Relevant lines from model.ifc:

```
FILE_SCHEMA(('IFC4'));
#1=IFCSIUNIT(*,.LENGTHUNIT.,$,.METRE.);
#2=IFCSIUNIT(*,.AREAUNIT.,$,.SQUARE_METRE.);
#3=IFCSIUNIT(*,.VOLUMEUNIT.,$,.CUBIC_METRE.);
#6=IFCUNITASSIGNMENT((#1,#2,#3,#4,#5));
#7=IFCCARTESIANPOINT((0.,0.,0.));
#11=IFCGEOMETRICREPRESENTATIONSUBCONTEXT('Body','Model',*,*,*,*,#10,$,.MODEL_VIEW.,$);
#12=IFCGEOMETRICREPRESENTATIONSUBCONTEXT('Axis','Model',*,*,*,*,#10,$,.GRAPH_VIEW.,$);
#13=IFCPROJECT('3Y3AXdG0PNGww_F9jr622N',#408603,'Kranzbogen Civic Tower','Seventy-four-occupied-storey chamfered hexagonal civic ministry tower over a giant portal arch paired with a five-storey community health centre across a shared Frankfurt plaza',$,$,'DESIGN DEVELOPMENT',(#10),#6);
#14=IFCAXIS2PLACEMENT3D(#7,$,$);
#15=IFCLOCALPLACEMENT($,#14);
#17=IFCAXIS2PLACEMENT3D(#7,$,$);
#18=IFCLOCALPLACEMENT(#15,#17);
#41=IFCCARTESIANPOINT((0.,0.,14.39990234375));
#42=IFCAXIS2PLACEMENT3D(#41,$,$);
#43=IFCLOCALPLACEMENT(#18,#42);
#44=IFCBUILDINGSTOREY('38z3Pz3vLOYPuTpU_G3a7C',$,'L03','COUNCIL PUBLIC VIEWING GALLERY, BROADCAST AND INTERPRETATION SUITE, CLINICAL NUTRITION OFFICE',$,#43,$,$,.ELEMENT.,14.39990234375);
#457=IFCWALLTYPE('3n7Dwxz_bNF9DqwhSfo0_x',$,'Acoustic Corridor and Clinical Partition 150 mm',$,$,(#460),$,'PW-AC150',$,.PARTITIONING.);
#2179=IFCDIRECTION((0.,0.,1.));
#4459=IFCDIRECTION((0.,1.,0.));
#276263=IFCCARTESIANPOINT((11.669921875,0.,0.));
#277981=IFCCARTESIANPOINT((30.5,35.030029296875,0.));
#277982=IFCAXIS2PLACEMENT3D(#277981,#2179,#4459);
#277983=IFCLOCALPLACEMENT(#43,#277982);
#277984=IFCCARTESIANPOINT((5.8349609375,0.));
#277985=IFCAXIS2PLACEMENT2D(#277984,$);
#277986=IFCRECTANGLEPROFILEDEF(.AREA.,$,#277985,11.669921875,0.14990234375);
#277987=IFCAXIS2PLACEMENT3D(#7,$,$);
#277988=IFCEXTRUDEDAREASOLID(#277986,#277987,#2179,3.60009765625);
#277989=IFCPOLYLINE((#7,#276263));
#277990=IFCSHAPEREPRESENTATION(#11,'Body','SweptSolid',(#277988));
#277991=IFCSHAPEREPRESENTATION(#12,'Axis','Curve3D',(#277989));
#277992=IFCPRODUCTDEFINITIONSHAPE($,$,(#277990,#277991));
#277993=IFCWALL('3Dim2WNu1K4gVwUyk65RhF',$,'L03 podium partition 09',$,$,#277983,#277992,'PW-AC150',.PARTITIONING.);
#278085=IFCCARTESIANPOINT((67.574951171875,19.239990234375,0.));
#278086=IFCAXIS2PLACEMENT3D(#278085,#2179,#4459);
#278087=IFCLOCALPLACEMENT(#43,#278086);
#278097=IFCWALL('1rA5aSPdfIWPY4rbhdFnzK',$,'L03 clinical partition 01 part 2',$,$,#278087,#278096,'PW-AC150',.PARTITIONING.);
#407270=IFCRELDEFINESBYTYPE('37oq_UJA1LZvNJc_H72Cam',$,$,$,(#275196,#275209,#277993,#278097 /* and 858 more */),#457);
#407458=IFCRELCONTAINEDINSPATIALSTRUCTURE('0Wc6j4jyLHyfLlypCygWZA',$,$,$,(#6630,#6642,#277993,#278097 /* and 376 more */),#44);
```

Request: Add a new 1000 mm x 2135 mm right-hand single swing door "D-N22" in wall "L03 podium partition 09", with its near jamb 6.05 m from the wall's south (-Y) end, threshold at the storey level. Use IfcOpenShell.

```python
import numpy as np
import ifcopenshell
import ifcopenshell.api.feature
import ifcopenshell.api.geometry
import ifcopenshell.api.root
import ifcopenshell.api.spatial
import ifcopenshell.geom
import ifcopenshell.util.element
import ifcopenshell.util.placement
import ifcopenshell.util.representation
import ifcopenshell.util.shape
import ifcopenshell.util.unit

model = ifcopenshell.open("model.ifc")
unit_scale = ifcopenshell.util.unit.calculate_unit_scale(model)
settings = ifcopenshell.geom.settings()


def volume(element):
    """Net volume in cubic metres, openings subtracted."""
    shape = ifcopenshell.geom.create_shape(settings, element)
    return ifcopenshell.util.shape.get_volume(shape.geometry)


wall = model.by_guid("3Dim2WNu1K4gVwUyk65RhF")
storey = ifcopenshell.util.element.get_container(wall, ifc_class="IfcBuildingStorey")
context = ifcopenshell.util.representation.get_context(model, "Model", "Body", "MODEL_VIEW")
before = volume(wall)

width, height, from_end, sill = 1, 2.135, 6.05, 0.0  # metres

# The wall runs along its own X axis, and the end named is its -X end.
wall_shape = ifcopenshell.geom.create_shape(settings, wall)
x, y, z = ifcopenshell.util.shape.get_vertices(wall_shape.geometry).T
start = x.min() + from_end
face, thickness = float(y.min()), float(y.max() - y.min())
wall_matrix = ifcopenshell.util.placement.get_local_placement(wall.ObjectPlacement)
level = ifcopenshell.util.placement.get_local_placement(storey.ObjectPlacement)[2, 3]


def in_wall(x, y):
    """Placement at x, y metres in the wall's axes, at sill height."""
    matrix = wall_matrix.copy()
    matrix[:, 3] = wall_matrix @ np.array([x / unit_scale, y / unit_scale, 0.0, 1.0])
    matrix[2, 3] = level + sill / unit_scale
    return matrix


# Opening: a box that overshoots both wall faces by 50 mm.
opening = ifcopenshell.api.root.create_entity(model, ifc_class="IfcOpeningElement", predefined_type="OPENING")
box = ifcopenshell.api.geometry.add_wall_representation(
    model, context=context, length=width, height=height, thickness=thickness + 0.1
)
ifcopenshell.api.geometry.assign_representation(model, product=opening, representation=box)
ifcopenshell.api.geometry.edit_object_placement(model, product=opening, matrix=in_wall(start, face - 0.05), is_si=False)
ifcopenshell.api.feature.add_feature(model, feature=opening, element=wall)

door = ifcopenshell.api.root.create_entity(model, ifc_class="IfcDoor", name="D-N22", predefined_type="DOOR")
door.OverallWidth, door.OverallHeight = width / unit_scale, height / unit_scale
door.OperationType = "SINGLE_SWING_RIGHT"
body = ifcopenshell.api.geometry.add_door_representation(
    model,
    context=context,
    overall_width=door.OverallWidth,
    overall_height=door.OverallHeight,
    operation_type="SINGLE_SWING_RIGHT",
    lining_properties={"LiningDepth": thickness / unit_scale, "ThresholdDepth": thickness / unit_scale},
)
ifcopenshell.api.geometry.assign_representation(model, product=door, representation=body)
ifcopenshell.api.spatial.assign_container(model, products=[door], relating_structure=storey)
ifcopenshell.api.feature.add_filling(model, opening=opening, element=door)

# The lining spans the wall, so the door starts at the wall face.
ifcopenshell.api.geometry.edit_object_placement(model, product=door, matrix=in_wall(start, face), is_si=False)

after = volume(wall)

print(f"wall volume {before:.3f} -> {after:.3f} m3")

model.write("model-out.ifc")
```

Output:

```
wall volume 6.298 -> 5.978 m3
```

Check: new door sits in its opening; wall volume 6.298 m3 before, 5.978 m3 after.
